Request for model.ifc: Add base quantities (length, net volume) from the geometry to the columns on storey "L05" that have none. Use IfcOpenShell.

First a look at what the model holds.

```python
import ifcopenshell
import ifcopenshell.util.element
import ifcopenshell.util.unit

model = ifcopenshell.open("model.ifc")
print(model.schema)
for unit_type in ("LENGTHUNIT", "AREAUNIT", "VOLUMEUNIT"):
    print(unit_type, ifcopenshell.util.unit.calculate_unit_scale(model, unit_type))
storey = next(s for s in model.by_type("IfcBuildingStorey") if s.Name == "L05")
columns = [e for e in ifcopenshell.util.element.get_decomposition(storey) if e.is_a("IfcColumn")]
for e in sorted(columns, key=lambda e: e.id()):
    print(e.id(), e.is_a(), e.Name, list(ifcopenshell.util.element.get_psets(e, qtos_only=True)), sep=" | ")
```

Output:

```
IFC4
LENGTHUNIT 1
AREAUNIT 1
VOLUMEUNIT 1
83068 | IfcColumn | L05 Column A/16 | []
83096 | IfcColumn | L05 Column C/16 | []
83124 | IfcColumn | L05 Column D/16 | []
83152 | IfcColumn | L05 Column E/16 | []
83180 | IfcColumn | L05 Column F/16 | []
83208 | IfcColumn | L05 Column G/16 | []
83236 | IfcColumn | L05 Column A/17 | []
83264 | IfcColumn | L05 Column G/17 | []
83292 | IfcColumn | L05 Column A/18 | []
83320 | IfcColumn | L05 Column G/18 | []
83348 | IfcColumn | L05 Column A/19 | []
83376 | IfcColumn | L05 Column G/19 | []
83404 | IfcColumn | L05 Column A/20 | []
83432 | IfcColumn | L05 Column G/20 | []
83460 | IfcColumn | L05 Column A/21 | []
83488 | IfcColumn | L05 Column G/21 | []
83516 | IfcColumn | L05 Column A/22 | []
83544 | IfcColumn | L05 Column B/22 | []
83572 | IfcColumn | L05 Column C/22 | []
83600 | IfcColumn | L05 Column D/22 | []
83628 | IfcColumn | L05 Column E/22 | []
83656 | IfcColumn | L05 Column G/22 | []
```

```python
import ifcopenshell
import ifcopenshell.api.pset
import ifcopenshell.geom
import ifcopenshell.util.element
import ifcopenshell.util.shape
import ifcopenshell.util.unit

model = ifcopenshell.open("model.ifc")
unit_scale = ifcopenshell.util.unit.calculate_unit_scale(model)
volume_scale = ifcopenshell.util.unit.calculate_unit_scale(model, "VOLUMEUNIT")
settings = ifcopenshell.geom.settings()

storey = next(s for s in model.by_type("IfcBuildingStorey") if s.Name == "L05")
columns = [e for e in ifcopenshell.util.element.get_decomposition(storey) if e.is_a("IfcColumn")]

for e in sorted(columns, key=lambda e: e.id()):
    if ifcopenshell.util.element.get_psets(e, qtos_only=True, should_inherit=False):
        continue
    # Geometry comes back in metres, in the element's own axes.
    shape = ifcopenshell.geom.create_shape(settings, e)
    values = {
        "Length": ifcopenshell.util.shape.get_z(shape.geometry) / unit_scale,
        "NetVolume": ifcopenshell.util.shape.get_volume(shape.geometry) / volume_scale,
    }
    qto = ifcopenshell.api.pset.add_qto(model, product=e, name="Qto_ColumnBaseQuantities")
    ifcopenshell.api.pset.edit_qto(model, qto=qto, properties=values)
    print(e.id(), {k: round(v, 3) for k, v in values.items()})

model.write("model_updated.ifc")
```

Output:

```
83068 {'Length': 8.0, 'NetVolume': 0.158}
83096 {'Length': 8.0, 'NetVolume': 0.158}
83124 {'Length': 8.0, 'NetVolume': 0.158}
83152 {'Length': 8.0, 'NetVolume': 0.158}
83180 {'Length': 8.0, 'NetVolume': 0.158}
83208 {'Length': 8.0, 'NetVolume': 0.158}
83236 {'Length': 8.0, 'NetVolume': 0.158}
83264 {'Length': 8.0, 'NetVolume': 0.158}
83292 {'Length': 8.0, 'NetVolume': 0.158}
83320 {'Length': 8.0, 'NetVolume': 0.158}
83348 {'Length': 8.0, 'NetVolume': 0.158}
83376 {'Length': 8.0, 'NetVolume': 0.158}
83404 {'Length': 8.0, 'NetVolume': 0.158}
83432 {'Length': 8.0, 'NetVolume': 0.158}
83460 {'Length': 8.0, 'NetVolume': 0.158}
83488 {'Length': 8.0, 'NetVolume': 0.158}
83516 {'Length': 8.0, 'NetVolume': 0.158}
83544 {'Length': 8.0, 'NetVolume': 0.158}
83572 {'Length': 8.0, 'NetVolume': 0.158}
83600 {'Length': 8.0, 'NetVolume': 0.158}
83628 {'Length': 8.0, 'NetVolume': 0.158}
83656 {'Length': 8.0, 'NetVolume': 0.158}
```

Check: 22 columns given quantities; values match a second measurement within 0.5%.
